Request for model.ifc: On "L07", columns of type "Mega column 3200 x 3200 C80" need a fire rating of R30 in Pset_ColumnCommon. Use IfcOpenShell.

First a look at what the model holds.

```python
import ifcopenshell
import ifcopenshell.util.element

model = ifcopenshell.open("model.ifc")
print(model.schema)
storey = next(s for s in model.by_type("IfcBuildingStorey") if s.Name == "L07")
columns = [e for e in ifcopenshell.util.element.get_decomposition(storey) if e.is_a("IfcColumn")]
seen = {}
for e in columns:
    element_type = ifcopenshell.util.element.get_type(e)
    key = (element_type.Name if element_type != e and element_type else None, ifcopenshell.util.element.get_pset(e, "Pset_ColumnCommon", "FireRating"))
    seen[key] = seen.get(key, 0) + 1
for (name, value), count in sorted(seen.items(), key=str):
    print(count, "x", name, "|", value)
```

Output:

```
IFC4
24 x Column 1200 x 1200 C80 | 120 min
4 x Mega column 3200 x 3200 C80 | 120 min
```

```python
import ifcopenshell
import ifcopenshell.api.pset
import ifcopenshell.util.element

model = ifcopenshell.open("model.ifc")

storey = next(s for s in model.by_type("IfcBuildingStorey") if s.Name == "L07")
columns = [e for e in ifcopenshell.util.element.get_decomposition(storey) if e.is_a("IfcColumn")]

count = 0
for e in columns:
    element_type = ifcopenshell.util.element.get_type(e)
    if element_type in (None, e) or element_type.Name != "Mega column 3200 x 3200 C80":
        continue
    found = ifcopenshell.util.element.get_pset(e, "Pset_ColumnCommon", should_inherit=False)
    if found:
        pset = model.by_id(found["id"])
        if len(ifcopenshell.util.element.get_elements_by_pset(pset)) > 1:
            pset = ifcopenshell.api.pset.unshare_pset(model, products=[e], pset=pset)[0]
    else:
        pset = ifcopenshell.api.pset.add_pset(model, product=e, name="Pset_ColumnCommon")
    ifcopenshell.api.pset.edit_pset(model, pset=pset, properties={"FireRating": "R30"})
    count += 1

print(count, "columns updated")

model.write("model-out.ifc")
```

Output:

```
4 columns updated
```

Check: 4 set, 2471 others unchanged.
